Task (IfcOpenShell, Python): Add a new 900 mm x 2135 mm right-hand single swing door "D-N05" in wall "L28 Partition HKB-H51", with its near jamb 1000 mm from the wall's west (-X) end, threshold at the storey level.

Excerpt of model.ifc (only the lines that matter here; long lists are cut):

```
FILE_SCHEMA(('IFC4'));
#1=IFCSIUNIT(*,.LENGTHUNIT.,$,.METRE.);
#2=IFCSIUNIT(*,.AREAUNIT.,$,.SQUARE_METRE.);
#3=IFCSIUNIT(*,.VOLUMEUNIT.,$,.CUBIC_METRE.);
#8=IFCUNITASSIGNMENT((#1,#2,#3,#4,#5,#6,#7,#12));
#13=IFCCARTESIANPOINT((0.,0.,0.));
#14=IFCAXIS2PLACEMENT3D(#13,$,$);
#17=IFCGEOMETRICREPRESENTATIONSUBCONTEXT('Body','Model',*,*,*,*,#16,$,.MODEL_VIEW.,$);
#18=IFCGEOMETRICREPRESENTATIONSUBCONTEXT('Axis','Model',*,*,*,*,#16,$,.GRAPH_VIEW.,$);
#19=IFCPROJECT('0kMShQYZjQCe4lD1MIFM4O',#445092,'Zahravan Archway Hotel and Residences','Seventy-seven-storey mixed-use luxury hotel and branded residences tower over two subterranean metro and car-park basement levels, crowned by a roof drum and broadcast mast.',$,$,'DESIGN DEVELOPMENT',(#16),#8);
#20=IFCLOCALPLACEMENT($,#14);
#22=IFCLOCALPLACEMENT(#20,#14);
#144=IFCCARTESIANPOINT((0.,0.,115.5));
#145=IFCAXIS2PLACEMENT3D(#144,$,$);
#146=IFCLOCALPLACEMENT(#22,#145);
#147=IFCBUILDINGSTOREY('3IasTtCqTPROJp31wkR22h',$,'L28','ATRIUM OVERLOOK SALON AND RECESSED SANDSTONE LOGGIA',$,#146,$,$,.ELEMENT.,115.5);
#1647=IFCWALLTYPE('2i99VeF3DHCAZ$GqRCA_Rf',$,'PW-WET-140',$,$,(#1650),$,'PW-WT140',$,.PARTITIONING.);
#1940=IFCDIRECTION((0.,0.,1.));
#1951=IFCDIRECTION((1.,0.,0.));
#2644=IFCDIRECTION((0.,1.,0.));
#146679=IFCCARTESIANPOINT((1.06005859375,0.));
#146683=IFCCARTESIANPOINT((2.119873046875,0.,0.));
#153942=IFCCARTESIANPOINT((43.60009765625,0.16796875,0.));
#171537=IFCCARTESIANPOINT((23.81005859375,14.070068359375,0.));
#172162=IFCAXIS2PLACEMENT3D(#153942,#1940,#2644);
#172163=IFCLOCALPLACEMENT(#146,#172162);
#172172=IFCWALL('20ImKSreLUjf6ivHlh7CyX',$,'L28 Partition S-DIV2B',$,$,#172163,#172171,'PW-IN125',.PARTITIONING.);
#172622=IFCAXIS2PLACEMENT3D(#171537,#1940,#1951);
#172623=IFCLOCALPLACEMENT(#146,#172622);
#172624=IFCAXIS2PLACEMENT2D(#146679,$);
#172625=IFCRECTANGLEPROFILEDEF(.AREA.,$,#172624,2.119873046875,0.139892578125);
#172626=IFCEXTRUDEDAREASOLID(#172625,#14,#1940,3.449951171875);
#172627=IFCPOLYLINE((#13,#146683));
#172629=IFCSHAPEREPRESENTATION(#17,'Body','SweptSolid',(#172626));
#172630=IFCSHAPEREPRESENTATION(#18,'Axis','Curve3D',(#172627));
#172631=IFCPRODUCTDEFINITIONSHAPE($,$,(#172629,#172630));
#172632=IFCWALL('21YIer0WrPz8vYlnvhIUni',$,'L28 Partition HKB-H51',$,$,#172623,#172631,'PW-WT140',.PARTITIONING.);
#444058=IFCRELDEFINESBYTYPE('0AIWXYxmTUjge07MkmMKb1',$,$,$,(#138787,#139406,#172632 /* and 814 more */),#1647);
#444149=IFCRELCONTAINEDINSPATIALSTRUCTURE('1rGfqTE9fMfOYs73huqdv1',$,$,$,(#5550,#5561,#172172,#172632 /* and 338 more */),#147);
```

```python
import numpy as np
import ifcopenshell
import ifcopenshell.api.feature
import ifcopenshell.api.geometry
import ifcopenshell.api.root
import ifcopenshell.api.spatial
import ifcopenshell.geom
import ifcopenshell.util.element
import ifcopenshell.util.placement
import ifcopenshell.util.representation
import ifcopenshell.util.shape
import ifcopenshell.util.unit

model = ifcopenshell.open("model.ifc")
unit_scale = ifcopenshell.util.unit.calculate_unit_scale(model)
settings = ifcopenshell.geom.settings()


def volume(element):
    """Net volume in cubic metres, openings subtracted."""
    shape = ifcopenshell.geom.create_shape(settings, element)
    return ifcopenshell.util.shape.get_volume(shape.geometry)


wall = model.by_guid("21YIer0WrPz8vYlnvhIUni")
storey = ifcopenshell.util.element.get_container(wall, ifc_class="IfcBuildingStorey")
context = ifcopenshell.util.representation.get_context(model, "Model", "Body", "MODEL_VIEW")
before = volume(wall)

width, height, from_end, sill = 0.9, 2.135, 1, 0.0  # metres

# The wall runs along its own X axis, and the end named is its -X end.
wall_shape = ifcopenshell.geom.create_shape(settings, wall)
x, y, z = ifcopenshell.util.shape.get_vertices(wall_shape.geometry).T
start = x.min() + from_end
face, thickness = float(y.min()), float(y.max() - y.min())
wall_matrix = ifcopenshell.util.placement.get_local_placement(wall.ObjectPlacement)
level = ifcopenshell.util.placement.get_local_placement(storey.ObjectPlacement)[2, 3]


def in_wall(x, y):
    """Placement at x, y metres in the wall's axes, at sill height."""
    matrix = wall_matrix.copy()
    matrix[:, 3] = wall_matrix @ np.array([x / unit_scale, y / unit_scale, 0.0, 1.0])
    matrix[2, 3] = level + sill / unit_scale
    return matrix


# Opening: a box that overshoots both wall faces by 50 mm.
opening = ifcopenshell.api.root.create_entity(model, ifc_class="IfcOpeningElement", predefined_type="OPENING")
box = ifcopenshell.api.geometry.add_wall_representation(
    model, context=context, length=width, height=height, thickness=thickness + 0.1
)
ifcopenshell.api.geometry.assign_representation(model, product=opening, representation=box)
ifcopenshell.api.geometry.edit_object_placement(model, product=opening, matrix=in_wall(start, face - 0.05), is_si=False)
ifcopenshell.api.feature.add_feature(model, feature=opening, element=wall)

door = ifcopenshell.api.root.create_entity(model, ifc_class="IfcDoor", name="D-N05", predefined_type="DOOR")
door.OverallWidth, door.OverallHeight = width / unit_scale, height / unit_scale
door.OperationType = "SINGLE_SWING_RIGHT"
body = ifcopenshell.api.geometry.add_door_representation(
    model,
    context=context,
    overall_width=door.OverallWidth,
    overall_height=door.OverallHeight,
    operation_type="SINGLE_SWING_RIGHT",
    lining_properties={"LiningDepth": thickness / unit_scale, "ThresholdDepth": thickness / unit_scale},
)
ifcopenshell.api.geometry.assign_representation(model, product=door, representation=body)
ifcopenshell.api.spatial.assign_container(model, products=[door], relating_structure=storey)
ifcopenshell.api.feature.add_filling(model, opening=opening, element=door)

# The lining spans the wall, so the door starts at the wall face.
ifcopenshell.api.geometry.edit_object_placement(model, product=door, matrix=in_wall(start, face), is_si=False)

after = volume(wall)

print(f"wall volume {before:.3f} -> {after:.3f} m3")

model.write("model_updated.ifc")
```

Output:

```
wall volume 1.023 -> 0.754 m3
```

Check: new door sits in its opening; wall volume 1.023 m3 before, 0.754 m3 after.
